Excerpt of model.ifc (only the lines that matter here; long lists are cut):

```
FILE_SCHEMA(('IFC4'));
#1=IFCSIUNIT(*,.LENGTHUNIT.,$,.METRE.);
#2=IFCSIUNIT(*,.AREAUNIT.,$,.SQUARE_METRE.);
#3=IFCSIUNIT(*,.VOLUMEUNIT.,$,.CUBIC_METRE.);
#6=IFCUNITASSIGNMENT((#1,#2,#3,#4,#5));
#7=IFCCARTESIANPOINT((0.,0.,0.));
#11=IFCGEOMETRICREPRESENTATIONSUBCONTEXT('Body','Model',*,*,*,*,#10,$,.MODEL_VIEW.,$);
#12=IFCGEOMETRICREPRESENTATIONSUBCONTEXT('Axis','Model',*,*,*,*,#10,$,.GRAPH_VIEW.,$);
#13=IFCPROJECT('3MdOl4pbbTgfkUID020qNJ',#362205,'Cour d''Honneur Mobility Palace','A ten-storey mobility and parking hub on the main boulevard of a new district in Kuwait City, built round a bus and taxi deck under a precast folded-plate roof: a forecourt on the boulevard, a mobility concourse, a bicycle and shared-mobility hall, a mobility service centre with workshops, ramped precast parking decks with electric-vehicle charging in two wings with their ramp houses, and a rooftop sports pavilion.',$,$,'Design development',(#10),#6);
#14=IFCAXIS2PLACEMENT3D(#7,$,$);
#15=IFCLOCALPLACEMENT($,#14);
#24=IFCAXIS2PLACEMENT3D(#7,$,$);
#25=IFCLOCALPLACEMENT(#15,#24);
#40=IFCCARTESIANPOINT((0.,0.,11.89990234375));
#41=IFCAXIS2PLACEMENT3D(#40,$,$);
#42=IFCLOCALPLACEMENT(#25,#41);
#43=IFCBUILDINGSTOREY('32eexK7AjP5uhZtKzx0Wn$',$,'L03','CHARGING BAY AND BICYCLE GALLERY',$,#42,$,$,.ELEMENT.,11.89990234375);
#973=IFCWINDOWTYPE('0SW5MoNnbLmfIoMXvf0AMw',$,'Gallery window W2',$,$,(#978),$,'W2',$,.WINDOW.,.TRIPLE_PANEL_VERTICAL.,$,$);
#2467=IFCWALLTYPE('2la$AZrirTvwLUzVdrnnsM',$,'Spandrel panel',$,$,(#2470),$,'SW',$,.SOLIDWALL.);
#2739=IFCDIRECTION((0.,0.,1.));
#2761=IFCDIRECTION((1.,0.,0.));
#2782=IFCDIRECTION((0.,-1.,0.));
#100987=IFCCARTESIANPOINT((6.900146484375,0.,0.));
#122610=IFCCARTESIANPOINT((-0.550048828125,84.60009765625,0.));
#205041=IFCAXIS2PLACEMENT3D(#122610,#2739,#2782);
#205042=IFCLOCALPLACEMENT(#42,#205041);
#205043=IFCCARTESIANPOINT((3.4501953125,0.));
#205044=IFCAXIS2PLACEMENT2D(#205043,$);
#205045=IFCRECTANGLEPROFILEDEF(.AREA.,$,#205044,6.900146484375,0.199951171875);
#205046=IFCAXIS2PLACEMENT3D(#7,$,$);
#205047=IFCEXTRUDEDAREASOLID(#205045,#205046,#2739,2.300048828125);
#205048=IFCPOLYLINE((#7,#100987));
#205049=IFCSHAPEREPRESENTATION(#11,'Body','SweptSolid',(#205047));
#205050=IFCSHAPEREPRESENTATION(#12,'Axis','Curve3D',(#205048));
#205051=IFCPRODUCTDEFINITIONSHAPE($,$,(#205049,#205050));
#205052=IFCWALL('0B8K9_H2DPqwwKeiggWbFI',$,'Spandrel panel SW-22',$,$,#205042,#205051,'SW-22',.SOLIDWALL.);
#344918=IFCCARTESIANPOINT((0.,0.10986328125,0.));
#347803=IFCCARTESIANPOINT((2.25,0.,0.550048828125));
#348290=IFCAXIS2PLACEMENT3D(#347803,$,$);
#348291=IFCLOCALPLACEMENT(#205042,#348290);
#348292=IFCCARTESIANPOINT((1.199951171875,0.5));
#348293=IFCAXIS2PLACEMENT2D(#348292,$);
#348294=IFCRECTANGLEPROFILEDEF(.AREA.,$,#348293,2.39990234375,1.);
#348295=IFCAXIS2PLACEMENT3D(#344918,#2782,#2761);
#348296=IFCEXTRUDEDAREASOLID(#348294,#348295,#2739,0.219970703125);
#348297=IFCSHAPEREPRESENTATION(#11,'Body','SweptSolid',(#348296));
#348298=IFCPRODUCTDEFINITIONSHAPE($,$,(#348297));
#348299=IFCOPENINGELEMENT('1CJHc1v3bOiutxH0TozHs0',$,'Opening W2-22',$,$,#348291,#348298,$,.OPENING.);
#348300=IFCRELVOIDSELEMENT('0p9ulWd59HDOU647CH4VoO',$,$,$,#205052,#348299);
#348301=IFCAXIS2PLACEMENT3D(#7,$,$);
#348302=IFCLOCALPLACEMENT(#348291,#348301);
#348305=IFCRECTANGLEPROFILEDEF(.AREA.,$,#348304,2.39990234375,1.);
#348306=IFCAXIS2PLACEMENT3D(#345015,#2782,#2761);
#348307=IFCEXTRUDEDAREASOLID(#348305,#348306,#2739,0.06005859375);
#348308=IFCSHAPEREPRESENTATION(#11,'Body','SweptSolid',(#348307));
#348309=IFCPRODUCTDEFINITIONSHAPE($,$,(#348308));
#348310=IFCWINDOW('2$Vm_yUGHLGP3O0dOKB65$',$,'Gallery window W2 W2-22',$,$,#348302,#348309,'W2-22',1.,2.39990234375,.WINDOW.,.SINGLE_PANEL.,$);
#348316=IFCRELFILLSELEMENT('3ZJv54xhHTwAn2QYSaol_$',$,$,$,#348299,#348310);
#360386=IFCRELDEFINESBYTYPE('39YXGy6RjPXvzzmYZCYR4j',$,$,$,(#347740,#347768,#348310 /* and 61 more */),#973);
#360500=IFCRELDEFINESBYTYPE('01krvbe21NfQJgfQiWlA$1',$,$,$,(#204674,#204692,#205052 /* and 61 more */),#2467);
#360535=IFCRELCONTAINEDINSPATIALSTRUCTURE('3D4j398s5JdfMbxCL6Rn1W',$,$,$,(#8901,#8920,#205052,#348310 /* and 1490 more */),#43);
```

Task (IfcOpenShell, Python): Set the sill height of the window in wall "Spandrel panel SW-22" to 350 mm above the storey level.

```python
import numpy as np
import ifcopenshell
import ifcopenshell.api.geometry
import ifcopenshell.geom
import ifcopenshell.util.element
import ifcopenshell.util.placement
import ifcopenshell.util.shape
import ifcopenshell.util.unit

model = ifcopenshell.open("model.ifc")
unit_scale = ifcopenshell.util.unit.calculate_unit_scale(model)

window = model.by_guid("2$Vm_yUGHLGP3O0dOKB65$")
opening = window.FillsVoids[0].RelatingOpeningElement
storey = ifcopenshell.util.element.get_container(window, ifc_class="IfcBuildingStorey")
level = ifcopenshell.util.placement.get_local_placement(storey.ObjectPlacement)[2, 3]

# The opening's origin need not be at the sill, so measure its lowest point.
shape = ifcopenshell.geom.create_shape(ifcopenshell.geom.settings(), opening)
bottom = ifcopenshell.util.shape.get_shape_bottom_elevation(shape, shape.geometry) / unit_scale
dz = level + 0.35 / unit_scale - bottom

shift = np.array([0.0, 0.0, dz])
# The window is placed relative to its opening, so it follows when the opening moves.
matrix = ifcopenshell.util.placement.get_local_placement(opening.ObjectPlacement)
matrix[:3, 3] += shift
ifcopenshell.api.geometry.edit_object_placement(
    model, product=opening, matrix=matrix, is_si=False, should_transform_children=True
)

print(f"moved by {dz * unit_scale:+.3f} m")

model.write("model_edited.ifc")
```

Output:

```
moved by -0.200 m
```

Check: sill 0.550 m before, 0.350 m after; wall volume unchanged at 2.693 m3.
